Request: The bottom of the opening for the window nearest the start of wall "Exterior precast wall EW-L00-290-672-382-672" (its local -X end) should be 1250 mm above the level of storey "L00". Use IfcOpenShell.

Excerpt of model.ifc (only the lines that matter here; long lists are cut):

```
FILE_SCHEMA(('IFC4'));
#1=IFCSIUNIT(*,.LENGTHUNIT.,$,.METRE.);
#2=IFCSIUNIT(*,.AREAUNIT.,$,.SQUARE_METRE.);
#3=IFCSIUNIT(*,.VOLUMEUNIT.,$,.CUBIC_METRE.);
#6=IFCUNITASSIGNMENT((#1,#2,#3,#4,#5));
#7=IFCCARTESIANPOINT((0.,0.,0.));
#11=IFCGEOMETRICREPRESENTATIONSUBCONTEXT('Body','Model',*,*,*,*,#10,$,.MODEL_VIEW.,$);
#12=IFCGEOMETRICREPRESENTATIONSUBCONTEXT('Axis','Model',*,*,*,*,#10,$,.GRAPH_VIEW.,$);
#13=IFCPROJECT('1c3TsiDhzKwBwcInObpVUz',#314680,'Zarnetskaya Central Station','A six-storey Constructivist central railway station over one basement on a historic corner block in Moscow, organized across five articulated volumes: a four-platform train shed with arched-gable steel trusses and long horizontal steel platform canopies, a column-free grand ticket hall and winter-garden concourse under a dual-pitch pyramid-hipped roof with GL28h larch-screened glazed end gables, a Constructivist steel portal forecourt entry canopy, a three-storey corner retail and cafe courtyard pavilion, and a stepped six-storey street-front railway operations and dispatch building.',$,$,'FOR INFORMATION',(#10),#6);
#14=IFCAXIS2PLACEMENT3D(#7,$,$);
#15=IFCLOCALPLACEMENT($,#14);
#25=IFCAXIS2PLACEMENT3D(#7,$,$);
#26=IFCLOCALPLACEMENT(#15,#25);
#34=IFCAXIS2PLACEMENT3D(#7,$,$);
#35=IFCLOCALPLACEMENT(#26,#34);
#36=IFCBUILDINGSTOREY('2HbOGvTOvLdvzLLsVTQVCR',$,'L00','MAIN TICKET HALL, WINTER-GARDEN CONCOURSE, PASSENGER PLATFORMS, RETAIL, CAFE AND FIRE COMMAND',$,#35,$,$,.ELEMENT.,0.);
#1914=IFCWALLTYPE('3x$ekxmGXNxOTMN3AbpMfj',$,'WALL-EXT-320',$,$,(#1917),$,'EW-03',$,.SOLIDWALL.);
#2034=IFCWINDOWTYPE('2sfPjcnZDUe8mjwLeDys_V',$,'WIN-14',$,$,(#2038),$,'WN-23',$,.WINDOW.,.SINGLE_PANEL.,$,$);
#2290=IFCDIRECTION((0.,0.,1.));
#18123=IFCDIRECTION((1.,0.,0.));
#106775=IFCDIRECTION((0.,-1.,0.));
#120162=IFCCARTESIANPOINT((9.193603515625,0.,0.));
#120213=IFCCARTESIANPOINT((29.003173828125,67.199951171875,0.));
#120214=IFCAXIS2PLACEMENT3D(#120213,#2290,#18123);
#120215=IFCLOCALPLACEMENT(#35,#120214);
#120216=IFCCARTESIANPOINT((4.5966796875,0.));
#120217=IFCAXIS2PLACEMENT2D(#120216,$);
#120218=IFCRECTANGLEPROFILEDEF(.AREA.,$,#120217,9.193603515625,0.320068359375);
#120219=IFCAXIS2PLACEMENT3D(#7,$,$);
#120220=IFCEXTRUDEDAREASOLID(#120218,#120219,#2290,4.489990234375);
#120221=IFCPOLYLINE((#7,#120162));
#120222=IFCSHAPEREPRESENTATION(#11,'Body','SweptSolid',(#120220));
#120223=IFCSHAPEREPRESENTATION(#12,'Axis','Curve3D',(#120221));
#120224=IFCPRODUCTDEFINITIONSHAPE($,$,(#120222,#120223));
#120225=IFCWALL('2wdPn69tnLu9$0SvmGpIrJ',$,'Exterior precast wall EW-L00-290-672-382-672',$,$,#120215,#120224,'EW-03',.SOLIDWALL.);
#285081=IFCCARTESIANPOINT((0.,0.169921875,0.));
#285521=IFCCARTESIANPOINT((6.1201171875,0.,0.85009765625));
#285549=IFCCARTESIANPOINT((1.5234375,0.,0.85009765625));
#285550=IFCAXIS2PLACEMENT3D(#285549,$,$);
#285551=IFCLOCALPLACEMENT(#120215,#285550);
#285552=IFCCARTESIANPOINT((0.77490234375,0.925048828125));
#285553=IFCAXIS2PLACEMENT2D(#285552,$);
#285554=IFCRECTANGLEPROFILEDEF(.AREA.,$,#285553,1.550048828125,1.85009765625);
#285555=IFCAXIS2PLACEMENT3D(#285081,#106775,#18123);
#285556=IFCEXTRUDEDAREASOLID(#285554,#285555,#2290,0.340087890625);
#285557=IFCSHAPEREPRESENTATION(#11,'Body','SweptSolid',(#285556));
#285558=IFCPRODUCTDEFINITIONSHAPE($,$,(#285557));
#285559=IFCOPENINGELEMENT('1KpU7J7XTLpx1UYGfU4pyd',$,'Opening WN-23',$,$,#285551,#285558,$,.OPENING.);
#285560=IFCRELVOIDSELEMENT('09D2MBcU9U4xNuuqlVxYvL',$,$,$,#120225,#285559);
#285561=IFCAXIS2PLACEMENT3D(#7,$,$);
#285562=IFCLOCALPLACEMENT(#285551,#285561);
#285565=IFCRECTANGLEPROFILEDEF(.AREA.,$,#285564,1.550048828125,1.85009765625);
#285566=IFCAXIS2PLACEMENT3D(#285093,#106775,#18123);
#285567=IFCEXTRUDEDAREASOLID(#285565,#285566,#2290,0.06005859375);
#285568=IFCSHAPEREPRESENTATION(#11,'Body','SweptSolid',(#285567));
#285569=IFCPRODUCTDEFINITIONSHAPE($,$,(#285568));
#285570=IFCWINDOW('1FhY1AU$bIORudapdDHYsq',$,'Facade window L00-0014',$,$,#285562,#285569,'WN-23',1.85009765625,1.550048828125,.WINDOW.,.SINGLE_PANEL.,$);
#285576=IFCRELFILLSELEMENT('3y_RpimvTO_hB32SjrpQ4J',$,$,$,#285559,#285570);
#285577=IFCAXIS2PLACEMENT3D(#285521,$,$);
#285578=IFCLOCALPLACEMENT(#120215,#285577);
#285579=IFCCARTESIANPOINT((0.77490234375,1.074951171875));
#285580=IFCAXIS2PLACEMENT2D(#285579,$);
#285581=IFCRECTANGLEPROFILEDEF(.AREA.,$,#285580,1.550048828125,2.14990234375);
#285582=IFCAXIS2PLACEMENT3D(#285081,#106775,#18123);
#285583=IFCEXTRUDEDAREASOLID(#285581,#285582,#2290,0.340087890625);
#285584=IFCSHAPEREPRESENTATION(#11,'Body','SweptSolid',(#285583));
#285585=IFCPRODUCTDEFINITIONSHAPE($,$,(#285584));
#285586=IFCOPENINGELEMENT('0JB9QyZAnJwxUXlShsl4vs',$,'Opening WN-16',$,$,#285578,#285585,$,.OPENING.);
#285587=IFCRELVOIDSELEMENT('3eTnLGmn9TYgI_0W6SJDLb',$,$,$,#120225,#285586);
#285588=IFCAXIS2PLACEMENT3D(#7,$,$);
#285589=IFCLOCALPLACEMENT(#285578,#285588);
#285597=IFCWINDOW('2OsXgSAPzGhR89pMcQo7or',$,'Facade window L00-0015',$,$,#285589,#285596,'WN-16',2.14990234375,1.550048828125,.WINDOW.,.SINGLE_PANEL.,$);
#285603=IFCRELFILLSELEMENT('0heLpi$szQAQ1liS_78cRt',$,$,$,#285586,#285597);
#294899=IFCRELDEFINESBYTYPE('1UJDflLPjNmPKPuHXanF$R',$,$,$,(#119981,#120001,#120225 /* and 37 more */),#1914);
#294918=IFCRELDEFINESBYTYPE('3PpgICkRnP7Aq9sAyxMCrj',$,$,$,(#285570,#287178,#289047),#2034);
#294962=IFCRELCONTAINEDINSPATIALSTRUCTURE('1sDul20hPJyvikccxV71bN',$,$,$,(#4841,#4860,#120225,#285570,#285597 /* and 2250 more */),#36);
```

```python
import numpy as np
import ifcopenshell
import ifcopenshell.api.geometry
import ifcopenshell.geom
import ifcopenshell.util.element
import ifcopenshell.util.placement
import ifcopenshell.util.shape
import ifcopenshell.util.unit

model = ifcopenshell.open("model.ifc")
unit_scale = ifcopenshell.util.unit.calculate_unit_scale(model)

window = model.by_guid("1FhY1AU$bIORudapdDHYsq")
opening = window.FillsVoids[0].RelatingOpeningElement
storey = ifcopenshell.util.element.get_container(window, ifc_class="IfcBuildingStorey")
level = ifcopenshell.util.placement.get_local_placement(storey.ObjectPlacement)[2, 3]

# The opening's origin need not be at the sill, so measure its lowest point.
shape = ifcopenshell.geom.create_shape(ifcopenshell.geom.settings(), opening)
bottom = ifcopenshell.util.shape.get_shape_bottom_elevation(shape, shape.geometry) / unit_scale
dz = level + 1.25 / unit_scale - bottom

shift = np.array([0.0, 0.0, dz])
# The window is placed relative to its opening, so it follows when the opening moves.
matrix = ifcopenshell.util.placement.get_local_placement(opening.ObjectPlacement)
matrix[:3, 3] += shift
ifcopenshell.api.geometry.edit_object_placement(
    model, product=opening, matrix=matrix, is_si=False, should_transform_children=True
)

print(f"moved by {dz * unit_scale:+.3f} m")

model.write("model_updated.ifc")
```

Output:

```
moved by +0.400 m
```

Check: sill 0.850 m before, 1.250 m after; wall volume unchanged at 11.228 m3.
